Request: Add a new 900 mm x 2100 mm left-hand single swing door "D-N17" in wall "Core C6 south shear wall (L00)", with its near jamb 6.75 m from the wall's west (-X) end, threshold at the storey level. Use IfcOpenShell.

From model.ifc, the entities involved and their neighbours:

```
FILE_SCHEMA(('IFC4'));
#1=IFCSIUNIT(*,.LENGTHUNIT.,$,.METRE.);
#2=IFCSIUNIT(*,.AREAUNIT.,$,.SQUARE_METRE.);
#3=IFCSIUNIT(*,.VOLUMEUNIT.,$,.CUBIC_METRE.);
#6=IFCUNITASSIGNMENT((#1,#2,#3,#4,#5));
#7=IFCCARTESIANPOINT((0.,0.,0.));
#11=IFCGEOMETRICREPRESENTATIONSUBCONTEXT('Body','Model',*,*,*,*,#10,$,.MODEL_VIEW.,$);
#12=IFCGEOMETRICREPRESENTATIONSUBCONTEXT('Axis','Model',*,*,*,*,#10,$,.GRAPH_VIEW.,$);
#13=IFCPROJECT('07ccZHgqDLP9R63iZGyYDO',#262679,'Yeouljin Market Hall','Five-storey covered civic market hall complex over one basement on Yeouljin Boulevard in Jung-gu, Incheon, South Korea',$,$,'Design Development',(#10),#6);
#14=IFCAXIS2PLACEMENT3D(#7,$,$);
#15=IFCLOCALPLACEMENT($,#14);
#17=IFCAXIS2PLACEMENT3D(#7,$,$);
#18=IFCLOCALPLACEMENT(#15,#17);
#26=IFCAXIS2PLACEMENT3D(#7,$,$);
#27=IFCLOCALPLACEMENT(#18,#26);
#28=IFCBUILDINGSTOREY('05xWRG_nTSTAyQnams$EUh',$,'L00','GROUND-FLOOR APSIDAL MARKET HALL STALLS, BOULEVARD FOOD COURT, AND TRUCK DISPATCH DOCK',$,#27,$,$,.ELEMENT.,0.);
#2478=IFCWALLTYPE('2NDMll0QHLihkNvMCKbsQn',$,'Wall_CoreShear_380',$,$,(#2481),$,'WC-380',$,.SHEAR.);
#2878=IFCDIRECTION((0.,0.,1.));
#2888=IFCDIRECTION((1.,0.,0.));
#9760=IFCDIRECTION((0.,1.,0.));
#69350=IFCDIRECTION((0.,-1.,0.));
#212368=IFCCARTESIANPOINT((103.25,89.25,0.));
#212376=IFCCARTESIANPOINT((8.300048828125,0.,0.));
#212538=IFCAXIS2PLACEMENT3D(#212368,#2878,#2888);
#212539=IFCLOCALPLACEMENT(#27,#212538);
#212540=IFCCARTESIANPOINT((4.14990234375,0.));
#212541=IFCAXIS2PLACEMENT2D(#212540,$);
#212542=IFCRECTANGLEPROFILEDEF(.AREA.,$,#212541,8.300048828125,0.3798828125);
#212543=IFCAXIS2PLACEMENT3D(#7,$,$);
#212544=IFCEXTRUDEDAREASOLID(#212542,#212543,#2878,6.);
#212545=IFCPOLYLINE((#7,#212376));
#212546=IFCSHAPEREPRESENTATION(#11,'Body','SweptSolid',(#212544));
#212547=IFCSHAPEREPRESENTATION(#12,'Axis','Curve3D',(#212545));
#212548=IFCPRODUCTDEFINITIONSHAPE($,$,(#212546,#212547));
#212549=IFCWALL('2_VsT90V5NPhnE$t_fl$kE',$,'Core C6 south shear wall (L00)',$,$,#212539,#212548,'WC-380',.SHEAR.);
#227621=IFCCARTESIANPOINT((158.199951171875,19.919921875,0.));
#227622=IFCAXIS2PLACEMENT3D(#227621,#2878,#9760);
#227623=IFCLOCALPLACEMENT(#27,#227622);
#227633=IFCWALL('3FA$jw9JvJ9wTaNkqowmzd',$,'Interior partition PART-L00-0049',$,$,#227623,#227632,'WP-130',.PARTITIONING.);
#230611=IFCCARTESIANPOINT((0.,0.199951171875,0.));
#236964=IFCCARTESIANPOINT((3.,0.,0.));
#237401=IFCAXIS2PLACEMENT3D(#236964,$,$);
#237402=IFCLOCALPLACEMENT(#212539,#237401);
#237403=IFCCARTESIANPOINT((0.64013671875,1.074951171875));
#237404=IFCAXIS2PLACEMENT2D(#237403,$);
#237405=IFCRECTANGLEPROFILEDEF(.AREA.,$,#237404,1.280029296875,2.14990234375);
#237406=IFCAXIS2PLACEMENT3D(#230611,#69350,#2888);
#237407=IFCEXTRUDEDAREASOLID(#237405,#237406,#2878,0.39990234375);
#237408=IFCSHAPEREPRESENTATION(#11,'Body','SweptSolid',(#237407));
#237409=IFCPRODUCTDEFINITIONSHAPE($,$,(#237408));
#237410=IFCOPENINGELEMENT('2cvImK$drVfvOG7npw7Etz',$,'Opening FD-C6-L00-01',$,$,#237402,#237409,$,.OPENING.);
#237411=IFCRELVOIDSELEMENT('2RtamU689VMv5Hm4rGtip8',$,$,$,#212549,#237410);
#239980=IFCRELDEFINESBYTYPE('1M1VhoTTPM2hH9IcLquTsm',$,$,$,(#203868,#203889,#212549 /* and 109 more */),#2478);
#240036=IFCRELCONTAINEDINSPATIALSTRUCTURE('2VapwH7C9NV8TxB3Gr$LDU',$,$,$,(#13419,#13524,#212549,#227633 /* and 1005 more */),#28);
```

```python
import numpy as np
import ifcopenshell
import ifcopenshell.api.feature
import ifcopenshell.api.geometry
import ifcopenshell.api.root
import ifcopenshell.api.spatial
import ifcopenshell.geom
import ifcopenshell.util.element
import ifcopenshell.util.placement
import ifcopenshell.util.representation
import ifcopenshell.util.shape
import ifcopenshell.util.unit

model = ifcopenshell.open("model.ifc")
unit_scale = ifcopenshell.util.unit.calculate_unit_scale(model)
settings = ifcopenshell.geom.settings()


def volume(element):
    """Net volume in cubic metres, openings subtracted."""
    shape = ifcopenshell.geom.create_shape(settings, element)
    return ifcopenshell.util.shape.get_volume(shape.geometry)


wall = model.by_guid("2_VsT90V5NPhnE$t_fl$kE")
storey = ifcopenshell.util.element.get_container(wall, ifc_class="IfcBuildingStorey")
context = ifcopenshell.util.representation.get_context(model, "Model", "Body", "MODEL_VIEW")
before = volume(wall)

width, height, from_end, sill = 0.9, 2.1, 6.75, 0.0  # metres

# The wall runs along its own X axis, and the end named is its -X end.
wall_shape = ifcopenshell.geom.create_shape(settings, wall)
x, y, z = ifcopenshell.util.shape.get_vertices(wall_shape.geometry).T
start = x.min() + from_end
face, thickness = float(y.min()), float(y.max() - y.min())
wall_matrix = ifcopenshell.util.placement.get_local_placement(wall.ObjectPlacement)
level = ifcopenshell.util.placement.get_local_placement(storey.ObjectPlacement)[2, 3]


def in_wall(x, y):
    """Placement at x, y metres in the wall's axes, at sill height."""
    matrix = wall_matrix.copy()
    matrix[:, 3] = wall_matrix @ np.array([x / unit_scale, y / unit_scale, 0.0, 1.0])
    matrix[2, 3] = level + sill / unit_scale
    return matrix


# Opening: a box that overshoots both wall faces by 50 mm.
opening = ifcopenshell.api.root.create_entity(model, ifc_class="IfcOpeningElement", predefined_type="OPENING")
box = ifcopenshell.api.geometry.add_wall_representation(
    model, context=context, length=width, height=height, thickness=thickness + 0.1
)
ifcopenshell.api.geometry.assign_representation(model, product=opening, representation=box)
ifcopenshell.api.geometry.edit_object_placement(model, product=opening, matrix=in_wall(start, face - 0.05), is_si=False)
ifcopenshell.api.feature.add_feature(model, feature=opening, element=wall)

door = ifcopenshell.api.root.create_entity(model, ifc_class="IfcDoor", name="D-N17", predefined_type="DOOR")
door.OverallWidth, door.OverallHeight = width / unit_scale, height / unit_scale
door.OperationType = "SINGLE_SWING_LEFT"
body = ifcopenshell.api.geometry.add_door_representation(
    model,
    context=context,
    overall_width=door.OverallWidth,
    overall_height=door.OverallHeight,
    operation_type="SINGLE_SWING_LEFT",
    lining_properties={"LiningDepth": thickness / unit_scale, "ThresholdDepth": thickness / unit_scale},
)
ifcopenshell.api.geometry.assign_representation(model, product=door, representation=body)
ifcopenshell.api.spatial.assign_container(model, products=[door], relating_structure=storey)
ifcopenshell.api.feature.add_filling(model, opening=opening, element=door)

# The lining spans the wall, so the door starts at the wall face.
ifcopenshell.api.geometry.edit_object_placement(model, product=door, matrix=in_wall(start, face), is_si=False)

after = volume(wall)

print(f"wall volume {before:.3f} -> {after:.3f} m3")

model.write("model_rev.ifc")
```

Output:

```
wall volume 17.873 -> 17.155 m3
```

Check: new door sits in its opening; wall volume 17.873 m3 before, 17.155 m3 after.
